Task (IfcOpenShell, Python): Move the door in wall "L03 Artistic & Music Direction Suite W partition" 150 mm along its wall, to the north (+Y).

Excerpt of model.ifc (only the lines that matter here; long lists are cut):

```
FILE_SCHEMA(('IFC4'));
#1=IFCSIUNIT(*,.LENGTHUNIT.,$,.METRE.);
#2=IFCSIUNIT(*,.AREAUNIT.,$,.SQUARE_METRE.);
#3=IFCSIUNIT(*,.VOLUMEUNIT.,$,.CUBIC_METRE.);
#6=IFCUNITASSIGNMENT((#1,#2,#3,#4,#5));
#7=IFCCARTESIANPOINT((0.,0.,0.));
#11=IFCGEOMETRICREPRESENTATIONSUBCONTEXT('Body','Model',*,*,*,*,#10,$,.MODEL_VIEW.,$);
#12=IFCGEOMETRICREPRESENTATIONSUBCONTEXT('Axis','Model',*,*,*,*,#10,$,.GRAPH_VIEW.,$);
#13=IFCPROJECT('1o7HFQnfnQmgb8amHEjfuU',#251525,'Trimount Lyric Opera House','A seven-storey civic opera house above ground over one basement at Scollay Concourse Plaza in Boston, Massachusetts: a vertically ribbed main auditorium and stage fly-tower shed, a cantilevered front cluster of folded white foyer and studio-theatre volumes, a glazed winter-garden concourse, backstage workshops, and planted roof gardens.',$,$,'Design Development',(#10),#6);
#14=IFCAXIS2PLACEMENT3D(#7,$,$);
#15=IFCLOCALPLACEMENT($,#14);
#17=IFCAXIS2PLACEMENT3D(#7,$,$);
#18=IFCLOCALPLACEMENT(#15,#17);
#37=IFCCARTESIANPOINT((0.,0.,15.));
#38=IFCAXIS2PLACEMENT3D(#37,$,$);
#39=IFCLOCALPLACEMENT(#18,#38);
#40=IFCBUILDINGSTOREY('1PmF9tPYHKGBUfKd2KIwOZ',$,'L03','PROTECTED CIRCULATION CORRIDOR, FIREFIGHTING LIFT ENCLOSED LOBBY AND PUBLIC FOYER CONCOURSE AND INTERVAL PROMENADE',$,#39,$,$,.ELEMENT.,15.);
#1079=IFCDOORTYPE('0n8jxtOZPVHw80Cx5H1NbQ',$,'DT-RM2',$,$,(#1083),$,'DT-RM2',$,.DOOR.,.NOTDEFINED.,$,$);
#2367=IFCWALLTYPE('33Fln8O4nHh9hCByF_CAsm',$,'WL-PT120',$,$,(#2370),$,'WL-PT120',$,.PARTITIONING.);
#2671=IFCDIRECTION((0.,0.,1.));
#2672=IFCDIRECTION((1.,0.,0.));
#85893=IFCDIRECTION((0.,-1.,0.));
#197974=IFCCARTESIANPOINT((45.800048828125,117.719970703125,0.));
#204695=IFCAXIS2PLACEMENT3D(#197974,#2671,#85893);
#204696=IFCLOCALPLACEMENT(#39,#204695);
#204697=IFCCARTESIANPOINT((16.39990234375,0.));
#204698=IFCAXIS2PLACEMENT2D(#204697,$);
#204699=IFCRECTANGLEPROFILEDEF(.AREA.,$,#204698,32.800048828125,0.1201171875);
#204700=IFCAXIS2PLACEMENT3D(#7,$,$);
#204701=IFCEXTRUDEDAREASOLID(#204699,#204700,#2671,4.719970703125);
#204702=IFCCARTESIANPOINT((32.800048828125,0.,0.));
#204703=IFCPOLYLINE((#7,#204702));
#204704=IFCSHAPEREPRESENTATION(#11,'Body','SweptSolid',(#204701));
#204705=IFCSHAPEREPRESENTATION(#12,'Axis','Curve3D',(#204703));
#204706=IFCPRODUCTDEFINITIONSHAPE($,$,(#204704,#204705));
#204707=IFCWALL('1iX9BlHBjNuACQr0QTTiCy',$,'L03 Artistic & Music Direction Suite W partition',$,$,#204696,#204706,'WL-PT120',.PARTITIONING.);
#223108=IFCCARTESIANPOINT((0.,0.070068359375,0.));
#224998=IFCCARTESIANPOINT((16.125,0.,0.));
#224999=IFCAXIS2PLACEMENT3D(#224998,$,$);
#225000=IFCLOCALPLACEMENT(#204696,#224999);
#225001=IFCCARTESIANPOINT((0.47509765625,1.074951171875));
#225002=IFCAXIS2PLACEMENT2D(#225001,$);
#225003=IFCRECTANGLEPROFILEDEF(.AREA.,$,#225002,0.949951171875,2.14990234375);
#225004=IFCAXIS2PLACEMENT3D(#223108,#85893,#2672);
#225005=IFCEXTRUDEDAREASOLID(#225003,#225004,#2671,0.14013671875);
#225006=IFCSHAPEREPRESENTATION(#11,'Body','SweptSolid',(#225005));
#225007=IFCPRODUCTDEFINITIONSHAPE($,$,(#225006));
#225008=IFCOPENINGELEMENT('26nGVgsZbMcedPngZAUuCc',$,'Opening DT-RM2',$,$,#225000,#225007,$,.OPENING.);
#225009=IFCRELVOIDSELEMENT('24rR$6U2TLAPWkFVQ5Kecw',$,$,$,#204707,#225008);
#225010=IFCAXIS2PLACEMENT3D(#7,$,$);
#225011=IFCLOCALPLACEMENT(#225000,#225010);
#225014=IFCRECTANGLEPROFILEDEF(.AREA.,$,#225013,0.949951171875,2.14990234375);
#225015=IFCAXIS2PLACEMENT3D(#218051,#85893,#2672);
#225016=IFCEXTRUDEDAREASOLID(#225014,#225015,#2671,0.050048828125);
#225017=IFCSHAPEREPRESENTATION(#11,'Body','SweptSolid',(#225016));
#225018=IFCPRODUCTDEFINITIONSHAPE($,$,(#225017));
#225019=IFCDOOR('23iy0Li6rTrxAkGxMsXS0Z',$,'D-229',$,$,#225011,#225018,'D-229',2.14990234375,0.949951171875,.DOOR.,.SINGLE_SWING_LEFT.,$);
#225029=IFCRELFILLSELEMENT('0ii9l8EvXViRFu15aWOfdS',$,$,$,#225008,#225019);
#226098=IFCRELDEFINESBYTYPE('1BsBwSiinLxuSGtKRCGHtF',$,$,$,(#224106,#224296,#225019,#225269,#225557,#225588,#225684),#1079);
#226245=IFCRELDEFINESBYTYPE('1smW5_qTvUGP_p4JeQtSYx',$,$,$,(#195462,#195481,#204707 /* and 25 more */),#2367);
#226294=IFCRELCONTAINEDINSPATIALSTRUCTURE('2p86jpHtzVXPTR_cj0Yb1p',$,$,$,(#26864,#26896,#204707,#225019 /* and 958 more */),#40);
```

```python
import ifcopenshell
import ifcopenshell.api.geometry
import ifcopenshell.util.placement
import ifcopenshell.util.unit

model = ifcopenshell.open("model.ifc")
unit_scale = ifcopenshell.util.unit.calculate_unit_scale(model)

door = model.by_guid("23iy0Li6rTrxAkGxMsXS0Z")
opening = door.FillsVoids[0].RelatingOpeningElement
wall = opening.VoidsElements[0].RelatingBuildingElement

wall_matrix = ifcopenshell.util.placement.get_local_placement(wall.ObjectPlacement)
shift = wall_matrix[:3, 0] * -0.15 / unit_scale
before = ifcopenshell.util.placement.get_local_placement(door.ObjectPlacement)[:3, 3].copy()

# The door is placed relative to its opening, so it follows when the opening moves.
matrix = ifcopenshell.util.placement.get_local_placement(opening.ObjectPlacement)
matrix[:3, 3] += shift
ifcopenshell.api.geometry.edit_object_placement(
    model, product=opening, matrix=matrix, is_si=False, should_transform_children=True
)

after = ifcopenshell.util.placement.get_local_placement(door.ObjectPlacement)[:3, 3]
print("door moved by", (after - before).round(3) + 0.0)

model.write("model-out.ifc")
```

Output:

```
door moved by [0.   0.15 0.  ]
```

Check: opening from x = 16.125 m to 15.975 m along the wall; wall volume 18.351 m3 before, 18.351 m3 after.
